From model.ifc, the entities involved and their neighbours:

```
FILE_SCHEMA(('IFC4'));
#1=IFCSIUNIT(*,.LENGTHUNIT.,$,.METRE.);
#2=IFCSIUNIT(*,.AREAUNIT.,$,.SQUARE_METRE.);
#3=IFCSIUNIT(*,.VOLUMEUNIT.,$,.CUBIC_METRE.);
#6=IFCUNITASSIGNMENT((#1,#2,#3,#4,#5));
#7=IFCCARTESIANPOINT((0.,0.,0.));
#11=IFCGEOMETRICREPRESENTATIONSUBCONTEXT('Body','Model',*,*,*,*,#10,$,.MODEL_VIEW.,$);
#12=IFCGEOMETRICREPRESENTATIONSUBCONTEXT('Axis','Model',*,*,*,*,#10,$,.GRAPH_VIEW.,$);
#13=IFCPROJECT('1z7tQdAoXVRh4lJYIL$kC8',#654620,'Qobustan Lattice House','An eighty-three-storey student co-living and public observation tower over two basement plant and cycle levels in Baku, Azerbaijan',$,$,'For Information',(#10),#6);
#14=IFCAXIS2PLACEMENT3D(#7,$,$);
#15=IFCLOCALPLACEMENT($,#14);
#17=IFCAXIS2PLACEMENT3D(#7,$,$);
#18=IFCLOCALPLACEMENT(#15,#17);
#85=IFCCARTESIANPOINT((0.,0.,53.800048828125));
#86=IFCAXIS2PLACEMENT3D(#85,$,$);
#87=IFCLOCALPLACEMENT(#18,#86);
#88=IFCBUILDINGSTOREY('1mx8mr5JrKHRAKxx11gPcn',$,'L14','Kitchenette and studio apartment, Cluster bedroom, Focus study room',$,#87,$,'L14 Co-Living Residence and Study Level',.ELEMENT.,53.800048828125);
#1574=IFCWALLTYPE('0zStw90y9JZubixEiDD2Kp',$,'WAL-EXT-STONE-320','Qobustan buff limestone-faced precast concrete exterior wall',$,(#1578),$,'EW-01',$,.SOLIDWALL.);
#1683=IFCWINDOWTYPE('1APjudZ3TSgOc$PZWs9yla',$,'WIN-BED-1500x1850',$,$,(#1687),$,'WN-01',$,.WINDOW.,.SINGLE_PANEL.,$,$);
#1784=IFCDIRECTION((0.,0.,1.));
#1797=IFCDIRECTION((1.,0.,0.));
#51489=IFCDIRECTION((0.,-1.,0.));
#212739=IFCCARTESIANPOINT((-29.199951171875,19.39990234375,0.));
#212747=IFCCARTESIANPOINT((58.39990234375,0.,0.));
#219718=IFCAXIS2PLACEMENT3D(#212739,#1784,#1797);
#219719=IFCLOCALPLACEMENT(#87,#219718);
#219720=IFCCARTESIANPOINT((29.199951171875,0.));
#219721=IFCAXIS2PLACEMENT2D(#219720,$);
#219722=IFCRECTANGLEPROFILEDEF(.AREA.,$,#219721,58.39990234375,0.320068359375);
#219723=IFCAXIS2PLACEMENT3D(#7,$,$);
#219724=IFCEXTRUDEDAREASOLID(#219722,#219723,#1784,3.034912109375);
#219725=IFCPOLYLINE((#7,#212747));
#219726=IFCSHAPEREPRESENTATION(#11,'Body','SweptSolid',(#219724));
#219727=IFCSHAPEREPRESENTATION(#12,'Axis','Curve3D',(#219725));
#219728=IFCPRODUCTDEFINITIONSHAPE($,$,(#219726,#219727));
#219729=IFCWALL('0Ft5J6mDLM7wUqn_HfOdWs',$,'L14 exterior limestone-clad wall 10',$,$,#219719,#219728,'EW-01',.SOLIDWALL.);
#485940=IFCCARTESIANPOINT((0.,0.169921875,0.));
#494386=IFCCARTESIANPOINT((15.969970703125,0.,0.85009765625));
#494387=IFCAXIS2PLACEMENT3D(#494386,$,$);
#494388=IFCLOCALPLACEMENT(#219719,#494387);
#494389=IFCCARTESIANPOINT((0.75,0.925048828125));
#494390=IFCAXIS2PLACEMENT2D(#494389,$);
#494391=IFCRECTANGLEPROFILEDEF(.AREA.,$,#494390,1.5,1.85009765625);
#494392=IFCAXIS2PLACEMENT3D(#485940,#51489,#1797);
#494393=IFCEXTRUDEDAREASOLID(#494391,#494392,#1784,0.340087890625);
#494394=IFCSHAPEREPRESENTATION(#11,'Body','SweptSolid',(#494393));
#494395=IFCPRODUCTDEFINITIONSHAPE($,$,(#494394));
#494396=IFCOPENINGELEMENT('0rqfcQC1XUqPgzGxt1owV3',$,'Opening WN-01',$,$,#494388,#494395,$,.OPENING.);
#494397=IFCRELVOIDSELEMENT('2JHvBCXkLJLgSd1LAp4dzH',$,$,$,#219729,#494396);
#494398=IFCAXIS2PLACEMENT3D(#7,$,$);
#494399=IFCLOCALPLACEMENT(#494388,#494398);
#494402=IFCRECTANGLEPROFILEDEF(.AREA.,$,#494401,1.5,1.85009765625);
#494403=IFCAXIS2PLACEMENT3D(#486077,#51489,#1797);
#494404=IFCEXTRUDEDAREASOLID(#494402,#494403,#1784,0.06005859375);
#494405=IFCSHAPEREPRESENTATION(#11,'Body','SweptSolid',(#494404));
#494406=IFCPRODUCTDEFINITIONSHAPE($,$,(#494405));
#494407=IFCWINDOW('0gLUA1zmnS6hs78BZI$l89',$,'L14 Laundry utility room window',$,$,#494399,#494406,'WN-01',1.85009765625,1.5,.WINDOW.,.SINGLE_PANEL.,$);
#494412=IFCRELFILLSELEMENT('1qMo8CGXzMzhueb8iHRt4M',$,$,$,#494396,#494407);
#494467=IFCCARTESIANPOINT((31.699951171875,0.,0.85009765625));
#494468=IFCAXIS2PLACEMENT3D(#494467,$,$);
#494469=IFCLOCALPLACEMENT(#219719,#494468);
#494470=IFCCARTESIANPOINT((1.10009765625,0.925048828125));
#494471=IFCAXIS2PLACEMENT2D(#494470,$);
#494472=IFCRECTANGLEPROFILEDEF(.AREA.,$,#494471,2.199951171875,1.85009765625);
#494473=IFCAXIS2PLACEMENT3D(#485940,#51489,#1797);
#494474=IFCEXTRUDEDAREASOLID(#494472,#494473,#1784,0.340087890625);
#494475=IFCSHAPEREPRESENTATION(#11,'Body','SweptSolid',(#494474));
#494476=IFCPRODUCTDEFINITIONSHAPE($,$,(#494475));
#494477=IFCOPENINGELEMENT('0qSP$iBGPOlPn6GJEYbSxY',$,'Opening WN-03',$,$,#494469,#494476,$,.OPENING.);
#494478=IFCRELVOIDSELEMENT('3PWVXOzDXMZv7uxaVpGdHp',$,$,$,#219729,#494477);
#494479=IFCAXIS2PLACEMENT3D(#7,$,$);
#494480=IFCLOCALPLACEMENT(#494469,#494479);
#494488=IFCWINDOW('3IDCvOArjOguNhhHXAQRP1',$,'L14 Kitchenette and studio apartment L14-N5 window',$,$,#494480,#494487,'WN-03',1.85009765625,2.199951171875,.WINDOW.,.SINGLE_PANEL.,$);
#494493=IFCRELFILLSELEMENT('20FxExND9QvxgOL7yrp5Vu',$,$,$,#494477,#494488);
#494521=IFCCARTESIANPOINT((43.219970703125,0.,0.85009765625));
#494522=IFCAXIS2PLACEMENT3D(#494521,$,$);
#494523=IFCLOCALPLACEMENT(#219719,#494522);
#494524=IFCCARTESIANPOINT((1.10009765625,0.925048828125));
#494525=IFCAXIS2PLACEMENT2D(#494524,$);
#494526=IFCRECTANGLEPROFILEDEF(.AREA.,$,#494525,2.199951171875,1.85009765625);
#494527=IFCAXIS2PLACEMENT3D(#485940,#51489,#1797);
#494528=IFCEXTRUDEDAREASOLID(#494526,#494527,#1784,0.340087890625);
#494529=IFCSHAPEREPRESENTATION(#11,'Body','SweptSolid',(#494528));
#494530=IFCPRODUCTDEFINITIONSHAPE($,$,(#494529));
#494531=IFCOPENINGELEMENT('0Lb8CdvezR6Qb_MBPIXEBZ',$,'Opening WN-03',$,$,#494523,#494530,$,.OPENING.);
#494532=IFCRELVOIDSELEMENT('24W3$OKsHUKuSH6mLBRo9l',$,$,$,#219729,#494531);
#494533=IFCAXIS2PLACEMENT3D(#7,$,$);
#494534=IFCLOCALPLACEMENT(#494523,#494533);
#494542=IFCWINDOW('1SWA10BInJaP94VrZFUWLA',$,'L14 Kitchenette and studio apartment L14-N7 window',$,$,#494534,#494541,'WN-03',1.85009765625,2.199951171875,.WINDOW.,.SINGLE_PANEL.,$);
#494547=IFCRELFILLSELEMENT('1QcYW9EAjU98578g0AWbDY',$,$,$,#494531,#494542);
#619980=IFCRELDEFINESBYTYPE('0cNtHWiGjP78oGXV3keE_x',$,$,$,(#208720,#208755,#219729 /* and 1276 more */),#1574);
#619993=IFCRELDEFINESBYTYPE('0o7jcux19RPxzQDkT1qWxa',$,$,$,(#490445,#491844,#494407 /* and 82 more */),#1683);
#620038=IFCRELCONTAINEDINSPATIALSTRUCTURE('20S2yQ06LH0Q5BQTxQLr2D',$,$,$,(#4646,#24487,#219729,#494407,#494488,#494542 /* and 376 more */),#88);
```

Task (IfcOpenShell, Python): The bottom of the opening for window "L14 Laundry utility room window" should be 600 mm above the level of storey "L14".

```python
import numpy as np
import ifcopenshell
import ifcopenshell.api.geometry
import ifcopenshell.geom
import ifcopenshell.util.element
import ifcopenshell.util.placement
import ifcopenshell.util.shape
import ifcopenshell.util.unit

model = ifcopenshell.open("model.ifc")
unit_scale = ifcopenshell.util.unit.calculate_unit_scale(model)

window = model.by_guid("0gLUA1zmnS6hs78BZI$l89")
opening = window.FillsVoids[0].RelatingOpeningElement
storey = ifcopenshell.util.element.get_container(window, ifc_class="IfcBuildingStorey")
level = ifcopenshell.util.placement.get_local_placement(storey.ObjectPlacement)[2, 3]

# The opening's origin need not be at the sill, so measure its lowest point.
shape = ifcopenshell.geom.create_shape(ifcopenshell.geom.settings(), opening)
bottom = ifcopenshell.util.shape.get_shape_bottom_elevation(shape, shape.geometry) / unit_scale
dz = level + 0.6 - bottom

shift = np.array([0.0, 0.0, dz])
# The window is placed relative to its opening, so it follows when the opening moves.
matrix = ifcopenshell.util.placement.get_local_placement(opening.ObjectPlacement)
matrix[:3, 3] += shift
ifcopenshell.api.geometry.edit_object_placement(
    model, product=opening, matrix=matrix, is_si=False, should_transform_children=True
)

print(f"moved by {dz * unit_scale:+.3f} m")

model.write("model_v2.ifc")
```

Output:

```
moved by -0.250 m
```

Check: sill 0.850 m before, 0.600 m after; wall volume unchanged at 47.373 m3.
